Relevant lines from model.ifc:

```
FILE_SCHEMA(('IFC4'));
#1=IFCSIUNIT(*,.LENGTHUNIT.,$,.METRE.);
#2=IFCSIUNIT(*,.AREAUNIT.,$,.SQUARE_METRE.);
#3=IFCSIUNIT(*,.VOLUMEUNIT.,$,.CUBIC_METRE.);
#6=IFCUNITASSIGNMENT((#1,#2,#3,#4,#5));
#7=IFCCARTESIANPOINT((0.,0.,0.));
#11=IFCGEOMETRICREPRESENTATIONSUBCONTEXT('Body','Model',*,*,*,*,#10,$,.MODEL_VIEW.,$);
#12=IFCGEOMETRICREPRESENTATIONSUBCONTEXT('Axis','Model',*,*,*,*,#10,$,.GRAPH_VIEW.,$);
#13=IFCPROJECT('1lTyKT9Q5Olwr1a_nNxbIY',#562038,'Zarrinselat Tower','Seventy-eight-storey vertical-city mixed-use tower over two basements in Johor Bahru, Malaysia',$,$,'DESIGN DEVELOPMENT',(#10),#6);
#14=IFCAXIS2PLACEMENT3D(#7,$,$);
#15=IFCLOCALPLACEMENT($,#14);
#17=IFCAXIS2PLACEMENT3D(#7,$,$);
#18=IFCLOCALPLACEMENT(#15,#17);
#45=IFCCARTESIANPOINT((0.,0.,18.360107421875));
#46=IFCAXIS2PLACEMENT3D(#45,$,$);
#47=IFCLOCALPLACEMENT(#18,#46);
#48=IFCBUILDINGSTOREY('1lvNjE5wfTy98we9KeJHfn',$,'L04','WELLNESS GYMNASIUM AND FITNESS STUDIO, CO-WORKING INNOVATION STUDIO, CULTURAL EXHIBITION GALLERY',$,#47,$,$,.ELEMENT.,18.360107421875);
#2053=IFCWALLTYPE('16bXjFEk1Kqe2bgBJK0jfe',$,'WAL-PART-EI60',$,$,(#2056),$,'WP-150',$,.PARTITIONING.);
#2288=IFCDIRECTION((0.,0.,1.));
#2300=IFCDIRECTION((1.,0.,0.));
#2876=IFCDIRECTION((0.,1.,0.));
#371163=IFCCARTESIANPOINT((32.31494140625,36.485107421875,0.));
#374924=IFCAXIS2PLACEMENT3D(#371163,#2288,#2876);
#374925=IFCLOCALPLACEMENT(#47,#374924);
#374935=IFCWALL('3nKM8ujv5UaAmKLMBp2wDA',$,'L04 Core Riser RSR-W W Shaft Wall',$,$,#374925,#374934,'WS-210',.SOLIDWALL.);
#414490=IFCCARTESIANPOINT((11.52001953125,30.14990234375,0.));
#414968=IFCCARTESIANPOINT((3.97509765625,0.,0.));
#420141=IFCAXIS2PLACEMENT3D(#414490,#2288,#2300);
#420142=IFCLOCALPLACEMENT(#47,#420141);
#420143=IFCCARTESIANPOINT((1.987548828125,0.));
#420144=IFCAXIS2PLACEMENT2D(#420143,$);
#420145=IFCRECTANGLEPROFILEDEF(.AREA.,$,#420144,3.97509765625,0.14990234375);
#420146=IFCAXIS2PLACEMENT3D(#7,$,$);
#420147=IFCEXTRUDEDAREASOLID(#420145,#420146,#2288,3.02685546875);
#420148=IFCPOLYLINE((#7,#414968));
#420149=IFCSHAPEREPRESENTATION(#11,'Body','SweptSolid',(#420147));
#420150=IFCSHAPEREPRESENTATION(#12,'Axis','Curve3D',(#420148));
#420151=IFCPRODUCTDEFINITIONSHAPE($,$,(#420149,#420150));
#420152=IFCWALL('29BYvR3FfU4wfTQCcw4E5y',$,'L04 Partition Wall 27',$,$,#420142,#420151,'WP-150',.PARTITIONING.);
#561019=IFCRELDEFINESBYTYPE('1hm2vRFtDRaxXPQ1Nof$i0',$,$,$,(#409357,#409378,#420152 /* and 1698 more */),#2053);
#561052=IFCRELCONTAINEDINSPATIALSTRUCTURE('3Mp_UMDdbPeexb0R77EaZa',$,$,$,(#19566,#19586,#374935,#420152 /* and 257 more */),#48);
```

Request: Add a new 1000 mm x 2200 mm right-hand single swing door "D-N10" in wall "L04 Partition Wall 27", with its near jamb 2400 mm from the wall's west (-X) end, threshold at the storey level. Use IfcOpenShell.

```python
import numpy as np
import ifcopenshell
import ifcopenshell.api.feature
import ifcopenshell.api.geometry
import ifcopenshell.api.root
import ifcopenshell.api.spatial
import ifcopenshell.geom
import ifcopenshell.util.element
import ifcopenshell.util.placement
import ifcopenshell.util.representation
import ifcopenshell.util.shape
import ifcopenshell.util.unit

model = ifcopenshell.open("model.ifc")
unit_scale = ifcopenshell.util.unit.calculate_unit_scale(model)
settings = ifcopenshell.geom.settings()


def volume(element):
    """Net volume in cubic metres, openings subtracted."""
    shape = ifcopenshell.geom.create_shape(settings, element)
    return ifcopenshell.util.shape.get_volume(shape.geometry)


wall = model.by_guid("29BYvR3FfU4wfTQCcw4E5y")
storey = ifcopenshell.util.element.get_container(wall, ifc_class="IfcBuildingStorey")
context = ifcopenshell.util.representation.get_context(model, "Model", "Body", "MODEL_VIEW")
before = volume(wall)

width, height, from_end, sill = 1, 2.2, 2.4, 0.0  # metres

# The wall runs along its own X axis, and the end named is its -X end.
wall_shape = ifcopenshell.geom.create_shape(settings, wall)
x, y, z = ifcopenshell.util.shape.get_vertices(wall_shape.geometry).T
start = x.min() + from_end
face, thickness = float(y.min()), float(y.max() - y.min())
wall_matrix = ifcopenshell.util.placement.get_local_placement(wall.ObjectPlacement)
level = ifcopenshell.util.placement.get_local_placement(storey.ObjectPlacement)[2, 3]


def in_wall(x, y):
    """Placement at x, y metres in the wall's axes, at sill height."""
    matrix = wall_matrix.copy()
    matrix[:, 3] = wall_matrix @ np.array([x / unit_scale, y / unit_scale, 0.0, 1.0])
    matrix[2, 3] = level + sill / unit_scale
    return matrix


# Opening: a box that overshoots both wall faces by 50 mm.
opening = ifcopenshell.api.root.create_entity(model, ifc_class="IfcOpeningElement", predefined_type="OPENING")
box = ifcopenshell.api.geometry.add_wall_representation(
    model, context=context, length=width, height=height, thickness=thickness + 0.1
)
ifcopenshell.api.geometry.assign_representation(model, product=opening, representation=box)
ifcopenshell.api.geometry.edit_object_placement(model, product=opening, matrix=in_wall(start, face - 0.05), is_si=False)
ifcopenshell.api.feature.add_feature(model, feature=opening, element=wall)

door = ifcopenshell.api.root.create_entity(model, ifc_class="IfcDoor", name="D-N10", predefined_type="DOOR")
door.OverallWidth, door.OverallHeight = width / unit_scale, height / unit_scale
door.OperationType = "SINGLE_SWING_RIGHT"
body = ifcopenshell.api.geometry.add_door_representation(
    model,
    context=context,
    overall_width=door.OverallWidth,
    overall_height=door.OverallHeight,
    operation_type="SINGLE_SWING_RIGHT",
    lining_properties={"LiningDepth": thickness / unit_scale, "ThresholdDepth": thickness / unit_scale},
)
ifcopenshell.api.geometry.assign_representation(model, product=door, representation=body)
ifcopenshell.api.spatial.assign_container(model, products=[door], relating_structure=storey)
ifcopenshell.api.feature.add_filling(model, opening=opening, element=door)

# The lining spans the wall, so the door starts at the wall face.
ifcopenshell.api.geometry.edit_object_placement(model, product=door, matrix=in_wall(start, face), is_si=False)

after = volume(wall)

print(f"wall volume {before:.3f} -> {after:.3f} m3")

model.write("model_v2.ifc")
```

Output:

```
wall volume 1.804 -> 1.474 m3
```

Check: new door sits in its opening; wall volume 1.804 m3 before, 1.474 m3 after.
